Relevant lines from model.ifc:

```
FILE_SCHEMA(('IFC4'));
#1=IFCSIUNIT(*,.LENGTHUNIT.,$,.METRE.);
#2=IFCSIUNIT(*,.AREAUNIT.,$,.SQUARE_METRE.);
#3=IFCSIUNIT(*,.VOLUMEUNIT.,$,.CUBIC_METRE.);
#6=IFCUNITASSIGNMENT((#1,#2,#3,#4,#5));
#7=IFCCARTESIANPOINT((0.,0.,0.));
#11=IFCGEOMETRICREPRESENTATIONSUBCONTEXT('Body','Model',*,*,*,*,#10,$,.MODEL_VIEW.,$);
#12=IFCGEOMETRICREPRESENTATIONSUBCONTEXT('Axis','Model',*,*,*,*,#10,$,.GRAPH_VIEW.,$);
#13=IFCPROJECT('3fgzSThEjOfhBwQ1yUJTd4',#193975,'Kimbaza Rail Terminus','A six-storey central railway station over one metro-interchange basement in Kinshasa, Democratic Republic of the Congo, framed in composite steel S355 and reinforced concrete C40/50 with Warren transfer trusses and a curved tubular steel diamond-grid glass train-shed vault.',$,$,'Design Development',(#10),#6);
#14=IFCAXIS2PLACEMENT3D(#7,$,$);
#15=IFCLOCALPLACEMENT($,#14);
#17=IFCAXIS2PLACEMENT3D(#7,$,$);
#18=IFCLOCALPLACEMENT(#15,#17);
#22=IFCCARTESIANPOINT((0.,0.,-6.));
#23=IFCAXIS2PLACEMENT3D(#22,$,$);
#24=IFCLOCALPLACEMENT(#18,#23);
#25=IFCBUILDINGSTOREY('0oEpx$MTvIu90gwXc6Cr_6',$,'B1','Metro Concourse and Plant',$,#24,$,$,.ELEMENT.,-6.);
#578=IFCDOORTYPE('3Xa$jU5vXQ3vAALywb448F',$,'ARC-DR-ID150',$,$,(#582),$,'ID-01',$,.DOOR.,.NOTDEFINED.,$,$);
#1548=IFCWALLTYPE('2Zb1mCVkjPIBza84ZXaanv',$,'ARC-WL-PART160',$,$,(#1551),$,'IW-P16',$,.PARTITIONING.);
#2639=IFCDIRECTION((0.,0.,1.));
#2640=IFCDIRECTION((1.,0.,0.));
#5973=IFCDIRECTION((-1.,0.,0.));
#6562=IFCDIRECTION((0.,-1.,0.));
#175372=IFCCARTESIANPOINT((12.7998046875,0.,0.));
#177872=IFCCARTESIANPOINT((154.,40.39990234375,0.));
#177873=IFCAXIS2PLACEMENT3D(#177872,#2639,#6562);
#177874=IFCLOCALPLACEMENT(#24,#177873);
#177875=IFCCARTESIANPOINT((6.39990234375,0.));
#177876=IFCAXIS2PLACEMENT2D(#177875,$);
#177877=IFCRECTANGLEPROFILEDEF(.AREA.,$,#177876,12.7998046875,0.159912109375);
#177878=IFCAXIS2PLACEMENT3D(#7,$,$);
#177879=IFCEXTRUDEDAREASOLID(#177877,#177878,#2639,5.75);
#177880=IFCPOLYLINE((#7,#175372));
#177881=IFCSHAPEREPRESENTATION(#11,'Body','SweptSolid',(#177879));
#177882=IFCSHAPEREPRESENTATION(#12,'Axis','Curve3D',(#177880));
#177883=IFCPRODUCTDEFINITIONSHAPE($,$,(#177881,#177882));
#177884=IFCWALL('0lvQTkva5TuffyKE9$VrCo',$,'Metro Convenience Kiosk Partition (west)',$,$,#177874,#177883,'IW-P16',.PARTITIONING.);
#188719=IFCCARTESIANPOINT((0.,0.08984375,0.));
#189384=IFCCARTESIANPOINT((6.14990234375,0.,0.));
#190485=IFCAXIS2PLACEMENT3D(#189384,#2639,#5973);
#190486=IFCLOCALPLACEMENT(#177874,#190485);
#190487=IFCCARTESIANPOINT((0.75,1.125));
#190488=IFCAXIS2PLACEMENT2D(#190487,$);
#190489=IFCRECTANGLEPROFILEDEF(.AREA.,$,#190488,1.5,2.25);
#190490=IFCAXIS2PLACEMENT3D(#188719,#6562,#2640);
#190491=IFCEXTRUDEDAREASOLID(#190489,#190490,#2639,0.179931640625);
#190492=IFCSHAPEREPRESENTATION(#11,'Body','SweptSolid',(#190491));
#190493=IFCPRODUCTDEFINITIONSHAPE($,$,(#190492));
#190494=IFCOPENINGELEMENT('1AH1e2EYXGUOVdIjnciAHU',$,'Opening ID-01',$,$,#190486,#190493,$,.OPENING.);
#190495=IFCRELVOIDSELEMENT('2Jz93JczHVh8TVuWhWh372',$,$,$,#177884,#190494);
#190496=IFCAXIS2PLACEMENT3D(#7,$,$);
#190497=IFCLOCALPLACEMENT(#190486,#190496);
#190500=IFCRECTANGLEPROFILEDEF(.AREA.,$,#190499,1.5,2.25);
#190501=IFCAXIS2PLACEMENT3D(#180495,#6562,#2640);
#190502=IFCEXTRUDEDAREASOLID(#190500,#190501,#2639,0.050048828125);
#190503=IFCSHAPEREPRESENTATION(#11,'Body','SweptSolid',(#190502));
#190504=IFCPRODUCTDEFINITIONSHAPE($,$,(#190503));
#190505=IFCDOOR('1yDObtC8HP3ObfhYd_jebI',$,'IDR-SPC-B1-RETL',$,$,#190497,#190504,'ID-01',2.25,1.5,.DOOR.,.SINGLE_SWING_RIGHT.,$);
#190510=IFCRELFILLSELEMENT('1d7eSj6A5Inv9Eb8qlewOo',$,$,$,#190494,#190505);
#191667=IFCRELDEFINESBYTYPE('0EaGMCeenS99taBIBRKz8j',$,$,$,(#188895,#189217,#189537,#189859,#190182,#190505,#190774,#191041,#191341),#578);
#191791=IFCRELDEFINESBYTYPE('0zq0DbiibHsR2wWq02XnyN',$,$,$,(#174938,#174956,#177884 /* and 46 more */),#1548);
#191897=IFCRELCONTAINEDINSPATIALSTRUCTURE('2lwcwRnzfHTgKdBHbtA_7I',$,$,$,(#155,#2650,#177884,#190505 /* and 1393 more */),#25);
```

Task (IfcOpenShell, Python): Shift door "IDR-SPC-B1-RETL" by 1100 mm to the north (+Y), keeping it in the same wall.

```python
import ifcopenshell
import ifcopenshell.api.geometry
import ifcopenshell.util.placement
import ifcopenshell.util.unit

model = ifcopenshell.open("model.ifc")
unit_scale = ifcopenshell.util.unit.calculate_unit_scale(model)

door = model.by_guid("1yDObtC8HP3ObfhYd_jebI")
opening = door.FillsVoids[0].RelatingOpeningElement
wall = opening.VoidsElements[0].RelatingBuildingElement

wall_matrix = ifcopenshell.util.placement.get_local_placement(wall.ObjectPlacement)
shift = wall_matrix[:3, 0] * -1.1 / unit_scale
before = ifcopenshell.util.placement.get_local_placement(door.ObjectPlacement)[:3, 3].copy()

# The door is placed relative to its opening, so it follows when the opening moves.
matrix = ifcopenshell.util.placement.get_local_placement(opening.ObjectPlacement)
matrix[:3, 3] += shift
ifcopenshell.api.geometry.edit_object_placement(
    model, product=opening, matrix=matrix, is_si=False, should_transform_children=True
)

after = ifcopenshell.util.placement.get_local_placement(door.ObjectPlacement)[:3, 3]
print("door moved by", (after - before).round(3) + 0.0)

model.write("model_updated.ifc")
```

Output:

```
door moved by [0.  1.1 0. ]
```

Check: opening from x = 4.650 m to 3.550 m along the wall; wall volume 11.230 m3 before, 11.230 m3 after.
